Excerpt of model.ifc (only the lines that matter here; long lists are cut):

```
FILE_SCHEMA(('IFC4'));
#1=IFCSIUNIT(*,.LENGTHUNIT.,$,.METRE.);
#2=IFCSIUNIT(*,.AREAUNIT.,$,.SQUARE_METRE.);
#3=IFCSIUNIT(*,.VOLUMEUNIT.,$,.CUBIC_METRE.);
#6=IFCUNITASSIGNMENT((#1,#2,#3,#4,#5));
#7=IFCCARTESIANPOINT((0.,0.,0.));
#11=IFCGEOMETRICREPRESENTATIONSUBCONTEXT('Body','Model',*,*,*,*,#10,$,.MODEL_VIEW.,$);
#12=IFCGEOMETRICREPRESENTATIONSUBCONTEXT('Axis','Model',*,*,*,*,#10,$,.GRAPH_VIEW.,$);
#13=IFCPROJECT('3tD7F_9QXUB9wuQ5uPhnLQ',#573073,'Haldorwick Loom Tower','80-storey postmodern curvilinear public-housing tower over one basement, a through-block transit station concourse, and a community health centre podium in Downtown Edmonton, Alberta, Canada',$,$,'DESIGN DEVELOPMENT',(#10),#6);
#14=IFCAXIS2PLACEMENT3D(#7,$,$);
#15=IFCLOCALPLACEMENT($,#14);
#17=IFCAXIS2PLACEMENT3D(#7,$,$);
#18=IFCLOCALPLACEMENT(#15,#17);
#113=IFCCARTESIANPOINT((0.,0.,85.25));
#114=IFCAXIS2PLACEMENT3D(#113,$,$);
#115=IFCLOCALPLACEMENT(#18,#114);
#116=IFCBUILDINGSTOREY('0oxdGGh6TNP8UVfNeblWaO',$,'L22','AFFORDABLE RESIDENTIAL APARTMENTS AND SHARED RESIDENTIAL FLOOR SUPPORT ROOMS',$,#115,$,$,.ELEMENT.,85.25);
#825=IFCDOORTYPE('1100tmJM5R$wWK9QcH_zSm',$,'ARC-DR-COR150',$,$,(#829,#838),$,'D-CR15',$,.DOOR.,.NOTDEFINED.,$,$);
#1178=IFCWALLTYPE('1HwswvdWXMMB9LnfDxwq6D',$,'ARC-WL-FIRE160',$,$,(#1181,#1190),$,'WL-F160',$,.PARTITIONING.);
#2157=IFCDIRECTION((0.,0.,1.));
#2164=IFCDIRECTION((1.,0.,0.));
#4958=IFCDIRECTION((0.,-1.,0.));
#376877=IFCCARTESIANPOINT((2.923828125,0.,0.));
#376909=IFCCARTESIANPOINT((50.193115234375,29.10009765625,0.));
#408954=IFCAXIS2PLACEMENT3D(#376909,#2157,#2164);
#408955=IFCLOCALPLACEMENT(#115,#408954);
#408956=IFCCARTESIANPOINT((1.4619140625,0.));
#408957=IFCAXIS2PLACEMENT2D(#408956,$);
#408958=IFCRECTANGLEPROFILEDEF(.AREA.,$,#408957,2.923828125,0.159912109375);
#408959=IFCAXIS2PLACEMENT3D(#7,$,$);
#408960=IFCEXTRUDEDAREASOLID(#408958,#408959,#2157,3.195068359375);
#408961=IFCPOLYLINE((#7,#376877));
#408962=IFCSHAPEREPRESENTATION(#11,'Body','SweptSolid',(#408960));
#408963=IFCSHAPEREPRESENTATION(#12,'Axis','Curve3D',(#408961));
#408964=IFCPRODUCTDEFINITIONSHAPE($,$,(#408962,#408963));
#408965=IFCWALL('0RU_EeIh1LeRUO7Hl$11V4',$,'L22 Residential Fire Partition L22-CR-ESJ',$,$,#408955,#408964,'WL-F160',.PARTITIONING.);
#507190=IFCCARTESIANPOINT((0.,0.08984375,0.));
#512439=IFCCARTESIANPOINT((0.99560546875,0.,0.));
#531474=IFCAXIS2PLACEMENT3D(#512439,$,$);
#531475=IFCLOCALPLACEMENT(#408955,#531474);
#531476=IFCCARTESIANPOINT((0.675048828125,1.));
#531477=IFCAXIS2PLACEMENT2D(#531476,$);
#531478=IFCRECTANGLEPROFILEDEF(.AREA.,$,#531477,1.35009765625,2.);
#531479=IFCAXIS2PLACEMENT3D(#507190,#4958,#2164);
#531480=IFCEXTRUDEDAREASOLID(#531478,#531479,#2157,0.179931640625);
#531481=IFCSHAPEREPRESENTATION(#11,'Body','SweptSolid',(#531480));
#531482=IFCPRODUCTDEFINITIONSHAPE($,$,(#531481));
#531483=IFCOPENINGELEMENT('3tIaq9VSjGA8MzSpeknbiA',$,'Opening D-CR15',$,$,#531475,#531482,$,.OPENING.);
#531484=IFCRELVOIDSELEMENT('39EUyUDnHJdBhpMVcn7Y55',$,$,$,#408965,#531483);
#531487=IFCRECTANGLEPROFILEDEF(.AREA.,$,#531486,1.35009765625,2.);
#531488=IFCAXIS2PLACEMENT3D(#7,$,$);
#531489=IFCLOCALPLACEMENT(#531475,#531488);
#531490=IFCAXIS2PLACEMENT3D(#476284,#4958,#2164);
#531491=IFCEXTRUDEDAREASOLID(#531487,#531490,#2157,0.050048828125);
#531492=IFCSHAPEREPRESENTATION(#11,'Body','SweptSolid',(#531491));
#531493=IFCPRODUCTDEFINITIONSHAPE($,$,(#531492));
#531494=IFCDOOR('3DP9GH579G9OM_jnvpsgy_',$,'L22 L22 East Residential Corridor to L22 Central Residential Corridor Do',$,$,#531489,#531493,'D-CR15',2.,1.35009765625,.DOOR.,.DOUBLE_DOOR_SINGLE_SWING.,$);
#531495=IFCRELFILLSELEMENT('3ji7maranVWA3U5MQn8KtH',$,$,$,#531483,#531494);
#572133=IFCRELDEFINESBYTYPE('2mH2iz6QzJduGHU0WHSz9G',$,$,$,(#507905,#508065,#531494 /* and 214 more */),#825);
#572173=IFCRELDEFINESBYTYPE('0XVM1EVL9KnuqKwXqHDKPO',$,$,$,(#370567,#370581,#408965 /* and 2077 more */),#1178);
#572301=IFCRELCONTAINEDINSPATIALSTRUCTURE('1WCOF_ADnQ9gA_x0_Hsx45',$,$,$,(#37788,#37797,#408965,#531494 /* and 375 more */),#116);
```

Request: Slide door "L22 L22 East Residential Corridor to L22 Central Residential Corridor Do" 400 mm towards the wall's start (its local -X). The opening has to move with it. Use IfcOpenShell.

```python
import ifcopenshell
import ifcopenshell.api.geometry
import ifcopenshell.util.placement
import ifcopenshell.util.unit

model = ifcopenshell.open("model.ifc")
unit_scale = ifcopenshell.util.unit.calculate_unit_scale(model)

door = model.by_guid("3DP9GH579G9OM_jnvpsgy_")
opening = door.FillsVoids[0].RelatingOpeningElement
wall = opening.VoidsElements[0].RelatingBuildingElement

wall_matrix = ifcopenshell.util.placement.get_local_placement(wall.ObjectPlacement)
shift = wall_matrix[:3, 0] * -0.4 / unit_scale
before = ifcopenshell.util.placement.get_local_placement(door.ObjectPlacement)[:3, 3].copy()

# The door is placed relative to its opening, so it follows when the opening moves.
matrix = ifcopenshell.util.placement.get_local_placement(opening.ObjectPlacement)
matrix[:3, 3] += shift
ifcopenshell.api.geometry.edit_object_placement(
    model, product=opening, matrix=matrix, is_si=False, should_transform_children=True
)

after = ifcopenshell.util.placement.get_local_placement(door.ObjectPlacement)[:3, 3]
print("door moved by", (after - before).round(3) + 0.0)

model.write("model_rev.ifc")
```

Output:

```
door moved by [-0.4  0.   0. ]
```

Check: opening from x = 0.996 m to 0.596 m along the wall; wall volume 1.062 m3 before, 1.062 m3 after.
